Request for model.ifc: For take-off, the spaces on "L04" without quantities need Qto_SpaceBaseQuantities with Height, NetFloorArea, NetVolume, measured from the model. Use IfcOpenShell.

First a look at what the model holds.

```python
import ifcopenshell
import ifcopenshell.util.element
import ifcopenshell.util.unit

model = ifcopenshell.open("model.ifc")
print(model.schema)
for unit_type in ("LENGTHUNIT", "AREAUNIT", "VOLUMEUNIT"):
    print(unit_type, ifcopenshell.util.unit.calculate_unit_scale(model, unit_type))
storey = next(s for s in model.by_type("IfcBuildingStorey") if s.Name == "L04")
spaces = [e for e in ifcopenshell.util.element.get_decomposition(storey) if e.is_a("IfcSpace")]
for e in sorted(spaces, key=lambda e: e.id()):
    print(e.id(), e.is_a(), e.Name, list(ifcopenshell.util.element.get_psets(e, qtos_only=True)), sep=" | ")
```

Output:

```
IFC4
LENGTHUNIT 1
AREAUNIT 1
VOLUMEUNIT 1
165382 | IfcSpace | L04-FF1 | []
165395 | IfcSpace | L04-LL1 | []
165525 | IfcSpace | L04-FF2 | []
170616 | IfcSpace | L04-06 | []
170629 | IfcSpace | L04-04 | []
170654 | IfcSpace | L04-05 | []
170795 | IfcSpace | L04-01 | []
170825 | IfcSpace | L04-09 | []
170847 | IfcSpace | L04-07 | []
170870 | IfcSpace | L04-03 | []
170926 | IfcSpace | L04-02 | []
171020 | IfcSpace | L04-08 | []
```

```python
import ifcopenshell
import ifcopenshell.api.pset
import ifcopenshell.geom
import ifcopenshell.util.element
import ifcopenshell.util.shape
import ifcopenshell.util.unit

model = ifcopenshell.open("model.ifc")
unit_scale = ifcopenshell.util.unit.calculate_unit_scale(model)
area_scale = ifcopenshell.util.unit.calculate_unit_scale(model, "AREAUNIT")
volume_scale = ifcopenshell.util.unit.calculate_unit_scale(model, "VOLUMEUNIT")
settings = ifcopenshell.geom.settings()

storey = next(s for s in model.by_type("IfcBuildingStorey") if s.Name == "L04")
spaces = [e for e in ifcopenshell.util.element.get_decomposition(storey) if e.is_a("IfcSpace")]

for e in sorted(spaces, key=lambda e: e.id()):
    if ifcopenshell.util.element.get_psets(e, qtos_only=True, should_inherit=False):
        continue
    # Geometry comes back in metres, in the element's own axes.
    shape = ifcopenshell.geom.create_shape(settings, e)
    values = {
        "Height": ifcopenshell.util.shape.get_z(shape.geometry) / unit_scale,
        "NetFloorArea": ifcopenshell.util.shape.get_footprint_area(shape.geometry) / area_scale,
        "NetVolume": ifcopenshell.util.shape.get_volume(shape.geometry) / volume_scale,
    }
    qto = ifcopenshell.api.pset.add_qto(model, product=e, name="Qto_SpaceBaseQuantities")
    ifcopenshell.api.pset.edit_qto(model, qto=qto, properties=values)
    print(e.id(), {k: round(v, 3) for k, v in values.items()})

model.write("model_rev.ifc")
```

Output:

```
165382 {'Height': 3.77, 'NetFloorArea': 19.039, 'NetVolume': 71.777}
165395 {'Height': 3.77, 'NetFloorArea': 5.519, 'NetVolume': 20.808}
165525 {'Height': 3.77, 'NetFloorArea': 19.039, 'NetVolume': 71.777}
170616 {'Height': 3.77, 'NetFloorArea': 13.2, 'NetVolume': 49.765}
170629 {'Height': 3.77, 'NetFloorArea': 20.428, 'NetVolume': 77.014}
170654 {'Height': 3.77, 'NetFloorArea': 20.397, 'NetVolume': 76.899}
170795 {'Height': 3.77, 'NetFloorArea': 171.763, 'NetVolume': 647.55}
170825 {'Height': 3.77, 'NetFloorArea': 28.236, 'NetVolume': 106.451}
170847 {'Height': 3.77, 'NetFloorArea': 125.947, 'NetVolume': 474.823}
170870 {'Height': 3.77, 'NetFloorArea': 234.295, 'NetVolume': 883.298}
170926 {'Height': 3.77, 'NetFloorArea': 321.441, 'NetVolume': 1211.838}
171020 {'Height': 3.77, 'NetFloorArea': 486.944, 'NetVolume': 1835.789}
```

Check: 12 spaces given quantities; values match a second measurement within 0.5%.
